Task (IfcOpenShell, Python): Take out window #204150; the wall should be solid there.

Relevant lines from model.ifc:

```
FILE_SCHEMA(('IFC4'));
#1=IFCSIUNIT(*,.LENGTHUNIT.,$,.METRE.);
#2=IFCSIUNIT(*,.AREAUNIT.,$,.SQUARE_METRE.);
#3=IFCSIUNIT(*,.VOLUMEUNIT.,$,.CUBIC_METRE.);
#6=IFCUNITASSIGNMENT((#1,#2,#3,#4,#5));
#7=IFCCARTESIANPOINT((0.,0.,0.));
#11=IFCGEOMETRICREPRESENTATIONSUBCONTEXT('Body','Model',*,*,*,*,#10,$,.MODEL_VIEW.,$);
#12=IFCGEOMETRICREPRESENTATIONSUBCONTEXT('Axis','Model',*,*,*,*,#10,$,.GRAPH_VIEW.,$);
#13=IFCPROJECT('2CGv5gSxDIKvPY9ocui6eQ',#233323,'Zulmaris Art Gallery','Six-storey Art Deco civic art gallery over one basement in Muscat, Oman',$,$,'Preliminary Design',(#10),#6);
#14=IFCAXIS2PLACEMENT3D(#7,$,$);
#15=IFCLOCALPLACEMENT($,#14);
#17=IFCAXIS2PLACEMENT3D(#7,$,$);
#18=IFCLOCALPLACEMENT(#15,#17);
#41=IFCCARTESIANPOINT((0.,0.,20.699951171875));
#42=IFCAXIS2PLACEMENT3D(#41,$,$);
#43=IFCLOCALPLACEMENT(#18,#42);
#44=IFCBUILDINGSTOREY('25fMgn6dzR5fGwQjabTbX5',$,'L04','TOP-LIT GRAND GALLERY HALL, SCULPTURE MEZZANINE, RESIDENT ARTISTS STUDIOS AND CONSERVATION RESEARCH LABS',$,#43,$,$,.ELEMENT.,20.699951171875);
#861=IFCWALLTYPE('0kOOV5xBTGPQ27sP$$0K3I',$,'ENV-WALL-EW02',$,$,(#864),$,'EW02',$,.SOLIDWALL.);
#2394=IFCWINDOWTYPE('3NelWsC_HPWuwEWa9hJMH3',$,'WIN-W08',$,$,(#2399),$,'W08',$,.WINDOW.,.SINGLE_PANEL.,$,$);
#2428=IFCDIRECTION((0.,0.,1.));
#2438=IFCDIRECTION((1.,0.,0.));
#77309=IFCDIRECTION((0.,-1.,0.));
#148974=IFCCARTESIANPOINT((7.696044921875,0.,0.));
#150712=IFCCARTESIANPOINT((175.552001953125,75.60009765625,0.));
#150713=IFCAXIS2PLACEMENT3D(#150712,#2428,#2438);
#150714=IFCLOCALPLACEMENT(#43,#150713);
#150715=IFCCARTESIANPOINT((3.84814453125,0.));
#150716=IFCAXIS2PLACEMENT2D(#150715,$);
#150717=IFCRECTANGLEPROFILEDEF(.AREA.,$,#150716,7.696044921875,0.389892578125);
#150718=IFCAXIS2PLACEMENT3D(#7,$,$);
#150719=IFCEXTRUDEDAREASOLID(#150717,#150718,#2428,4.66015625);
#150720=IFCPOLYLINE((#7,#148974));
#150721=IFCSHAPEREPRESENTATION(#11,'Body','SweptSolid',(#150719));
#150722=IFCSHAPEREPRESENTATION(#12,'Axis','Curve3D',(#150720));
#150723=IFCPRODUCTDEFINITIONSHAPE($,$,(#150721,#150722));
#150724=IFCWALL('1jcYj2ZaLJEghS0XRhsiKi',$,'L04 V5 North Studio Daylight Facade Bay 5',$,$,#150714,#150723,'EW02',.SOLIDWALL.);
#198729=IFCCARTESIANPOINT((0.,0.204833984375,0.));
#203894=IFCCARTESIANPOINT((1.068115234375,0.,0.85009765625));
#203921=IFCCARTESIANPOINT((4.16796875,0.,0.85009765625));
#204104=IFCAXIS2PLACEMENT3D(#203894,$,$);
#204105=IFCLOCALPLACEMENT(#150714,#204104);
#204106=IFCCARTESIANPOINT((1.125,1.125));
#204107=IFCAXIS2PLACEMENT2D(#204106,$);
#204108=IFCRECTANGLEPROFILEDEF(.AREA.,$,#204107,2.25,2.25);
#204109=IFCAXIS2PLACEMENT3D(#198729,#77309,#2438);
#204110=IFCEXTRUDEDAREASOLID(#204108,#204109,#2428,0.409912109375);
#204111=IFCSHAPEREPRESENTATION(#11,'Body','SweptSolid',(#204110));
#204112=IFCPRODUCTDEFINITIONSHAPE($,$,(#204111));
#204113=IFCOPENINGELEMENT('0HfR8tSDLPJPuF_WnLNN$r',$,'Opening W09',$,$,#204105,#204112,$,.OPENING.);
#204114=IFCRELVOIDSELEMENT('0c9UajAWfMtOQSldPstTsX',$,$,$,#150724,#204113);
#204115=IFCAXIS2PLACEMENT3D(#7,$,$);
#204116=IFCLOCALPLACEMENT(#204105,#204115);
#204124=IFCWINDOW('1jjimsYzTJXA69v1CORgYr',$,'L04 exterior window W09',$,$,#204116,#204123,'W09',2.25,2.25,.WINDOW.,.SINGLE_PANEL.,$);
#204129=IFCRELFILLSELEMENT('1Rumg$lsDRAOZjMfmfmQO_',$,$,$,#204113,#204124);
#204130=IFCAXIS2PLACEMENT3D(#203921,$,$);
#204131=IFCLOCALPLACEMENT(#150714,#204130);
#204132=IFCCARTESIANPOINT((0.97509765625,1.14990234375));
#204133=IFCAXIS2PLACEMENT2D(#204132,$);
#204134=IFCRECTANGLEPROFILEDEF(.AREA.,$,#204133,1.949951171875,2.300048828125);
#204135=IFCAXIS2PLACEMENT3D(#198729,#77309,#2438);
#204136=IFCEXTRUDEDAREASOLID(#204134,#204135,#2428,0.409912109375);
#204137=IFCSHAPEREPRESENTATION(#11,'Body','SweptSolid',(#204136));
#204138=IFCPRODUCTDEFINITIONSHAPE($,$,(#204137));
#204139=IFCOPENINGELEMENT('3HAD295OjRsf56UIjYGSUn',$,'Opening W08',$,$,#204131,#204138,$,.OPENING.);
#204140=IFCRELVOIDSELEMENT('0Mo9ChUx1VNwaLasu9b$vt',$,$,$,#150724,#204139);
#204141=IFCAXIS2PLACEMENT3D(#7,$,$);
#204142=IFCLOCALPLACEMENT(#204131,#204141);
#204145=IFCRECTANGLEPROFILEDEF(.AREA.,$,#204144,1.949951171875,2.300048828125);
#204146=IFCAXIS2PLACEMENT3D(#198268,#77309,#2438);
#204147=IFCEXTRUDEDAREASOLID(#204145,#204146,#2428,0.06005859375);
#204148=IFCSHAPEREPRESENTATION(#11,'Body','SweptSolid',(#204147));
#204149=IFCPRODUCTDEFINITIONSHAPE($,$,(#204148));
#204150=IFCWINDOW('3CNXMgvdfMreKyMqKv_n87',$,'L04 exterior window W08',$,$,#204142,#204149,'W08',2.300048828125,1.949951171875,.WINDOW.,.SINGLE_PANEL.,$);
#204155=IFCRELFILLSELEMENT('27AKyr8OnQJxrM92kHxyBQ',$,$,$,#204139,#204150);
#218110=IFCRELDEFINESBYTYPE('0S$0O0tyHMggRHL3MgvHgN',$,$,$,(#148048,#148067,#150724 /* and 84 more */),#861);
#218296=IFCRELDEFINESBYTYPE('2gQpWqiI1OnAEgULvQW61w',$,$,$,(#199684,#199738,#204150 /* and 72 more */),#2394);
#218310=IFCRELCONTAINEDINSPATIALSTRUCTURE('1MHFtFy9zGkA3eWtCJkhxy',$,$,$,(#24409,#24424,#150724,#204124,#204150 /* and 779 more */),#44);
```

```python
import ifcopenshell
import ifcopenshell.api.feature
import ifcopenshell.api.root
import ifcopenshell.geom
import ifcopenshell.util.shape

model = ifcopenshell.open("model.ifc")
settings = ifcopenshell.geom.settings()


def volume(element):
    """Net volume in cubic metres, openings subtracted."""
    shape = ifcopenshell.geom.create_shape(settings, element)
    return ifcopenshell.util.shape.get_volume(shape.geometry)


window = model.by_guid("3CNXMgvdfMreKyMqKv_n87")
opening = window.FillsVoids[0].RelatingOpeningElement
wall = opening.VoidsElements[0].RelatingBuildingElement
before = volume(wall)

ifcopenshell.api.root.remove_product(model, product=window)
ifcopenshell.api.feature.remove_feature(model, feature=opening)

after = volume(wall)

print(f"wall volume {before:.3f} -> {after:.3f} m3")

model.write("model-out.ifc")
```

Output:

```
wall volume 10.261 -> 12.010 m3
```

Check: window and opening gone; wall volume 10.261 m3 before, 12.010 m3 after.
